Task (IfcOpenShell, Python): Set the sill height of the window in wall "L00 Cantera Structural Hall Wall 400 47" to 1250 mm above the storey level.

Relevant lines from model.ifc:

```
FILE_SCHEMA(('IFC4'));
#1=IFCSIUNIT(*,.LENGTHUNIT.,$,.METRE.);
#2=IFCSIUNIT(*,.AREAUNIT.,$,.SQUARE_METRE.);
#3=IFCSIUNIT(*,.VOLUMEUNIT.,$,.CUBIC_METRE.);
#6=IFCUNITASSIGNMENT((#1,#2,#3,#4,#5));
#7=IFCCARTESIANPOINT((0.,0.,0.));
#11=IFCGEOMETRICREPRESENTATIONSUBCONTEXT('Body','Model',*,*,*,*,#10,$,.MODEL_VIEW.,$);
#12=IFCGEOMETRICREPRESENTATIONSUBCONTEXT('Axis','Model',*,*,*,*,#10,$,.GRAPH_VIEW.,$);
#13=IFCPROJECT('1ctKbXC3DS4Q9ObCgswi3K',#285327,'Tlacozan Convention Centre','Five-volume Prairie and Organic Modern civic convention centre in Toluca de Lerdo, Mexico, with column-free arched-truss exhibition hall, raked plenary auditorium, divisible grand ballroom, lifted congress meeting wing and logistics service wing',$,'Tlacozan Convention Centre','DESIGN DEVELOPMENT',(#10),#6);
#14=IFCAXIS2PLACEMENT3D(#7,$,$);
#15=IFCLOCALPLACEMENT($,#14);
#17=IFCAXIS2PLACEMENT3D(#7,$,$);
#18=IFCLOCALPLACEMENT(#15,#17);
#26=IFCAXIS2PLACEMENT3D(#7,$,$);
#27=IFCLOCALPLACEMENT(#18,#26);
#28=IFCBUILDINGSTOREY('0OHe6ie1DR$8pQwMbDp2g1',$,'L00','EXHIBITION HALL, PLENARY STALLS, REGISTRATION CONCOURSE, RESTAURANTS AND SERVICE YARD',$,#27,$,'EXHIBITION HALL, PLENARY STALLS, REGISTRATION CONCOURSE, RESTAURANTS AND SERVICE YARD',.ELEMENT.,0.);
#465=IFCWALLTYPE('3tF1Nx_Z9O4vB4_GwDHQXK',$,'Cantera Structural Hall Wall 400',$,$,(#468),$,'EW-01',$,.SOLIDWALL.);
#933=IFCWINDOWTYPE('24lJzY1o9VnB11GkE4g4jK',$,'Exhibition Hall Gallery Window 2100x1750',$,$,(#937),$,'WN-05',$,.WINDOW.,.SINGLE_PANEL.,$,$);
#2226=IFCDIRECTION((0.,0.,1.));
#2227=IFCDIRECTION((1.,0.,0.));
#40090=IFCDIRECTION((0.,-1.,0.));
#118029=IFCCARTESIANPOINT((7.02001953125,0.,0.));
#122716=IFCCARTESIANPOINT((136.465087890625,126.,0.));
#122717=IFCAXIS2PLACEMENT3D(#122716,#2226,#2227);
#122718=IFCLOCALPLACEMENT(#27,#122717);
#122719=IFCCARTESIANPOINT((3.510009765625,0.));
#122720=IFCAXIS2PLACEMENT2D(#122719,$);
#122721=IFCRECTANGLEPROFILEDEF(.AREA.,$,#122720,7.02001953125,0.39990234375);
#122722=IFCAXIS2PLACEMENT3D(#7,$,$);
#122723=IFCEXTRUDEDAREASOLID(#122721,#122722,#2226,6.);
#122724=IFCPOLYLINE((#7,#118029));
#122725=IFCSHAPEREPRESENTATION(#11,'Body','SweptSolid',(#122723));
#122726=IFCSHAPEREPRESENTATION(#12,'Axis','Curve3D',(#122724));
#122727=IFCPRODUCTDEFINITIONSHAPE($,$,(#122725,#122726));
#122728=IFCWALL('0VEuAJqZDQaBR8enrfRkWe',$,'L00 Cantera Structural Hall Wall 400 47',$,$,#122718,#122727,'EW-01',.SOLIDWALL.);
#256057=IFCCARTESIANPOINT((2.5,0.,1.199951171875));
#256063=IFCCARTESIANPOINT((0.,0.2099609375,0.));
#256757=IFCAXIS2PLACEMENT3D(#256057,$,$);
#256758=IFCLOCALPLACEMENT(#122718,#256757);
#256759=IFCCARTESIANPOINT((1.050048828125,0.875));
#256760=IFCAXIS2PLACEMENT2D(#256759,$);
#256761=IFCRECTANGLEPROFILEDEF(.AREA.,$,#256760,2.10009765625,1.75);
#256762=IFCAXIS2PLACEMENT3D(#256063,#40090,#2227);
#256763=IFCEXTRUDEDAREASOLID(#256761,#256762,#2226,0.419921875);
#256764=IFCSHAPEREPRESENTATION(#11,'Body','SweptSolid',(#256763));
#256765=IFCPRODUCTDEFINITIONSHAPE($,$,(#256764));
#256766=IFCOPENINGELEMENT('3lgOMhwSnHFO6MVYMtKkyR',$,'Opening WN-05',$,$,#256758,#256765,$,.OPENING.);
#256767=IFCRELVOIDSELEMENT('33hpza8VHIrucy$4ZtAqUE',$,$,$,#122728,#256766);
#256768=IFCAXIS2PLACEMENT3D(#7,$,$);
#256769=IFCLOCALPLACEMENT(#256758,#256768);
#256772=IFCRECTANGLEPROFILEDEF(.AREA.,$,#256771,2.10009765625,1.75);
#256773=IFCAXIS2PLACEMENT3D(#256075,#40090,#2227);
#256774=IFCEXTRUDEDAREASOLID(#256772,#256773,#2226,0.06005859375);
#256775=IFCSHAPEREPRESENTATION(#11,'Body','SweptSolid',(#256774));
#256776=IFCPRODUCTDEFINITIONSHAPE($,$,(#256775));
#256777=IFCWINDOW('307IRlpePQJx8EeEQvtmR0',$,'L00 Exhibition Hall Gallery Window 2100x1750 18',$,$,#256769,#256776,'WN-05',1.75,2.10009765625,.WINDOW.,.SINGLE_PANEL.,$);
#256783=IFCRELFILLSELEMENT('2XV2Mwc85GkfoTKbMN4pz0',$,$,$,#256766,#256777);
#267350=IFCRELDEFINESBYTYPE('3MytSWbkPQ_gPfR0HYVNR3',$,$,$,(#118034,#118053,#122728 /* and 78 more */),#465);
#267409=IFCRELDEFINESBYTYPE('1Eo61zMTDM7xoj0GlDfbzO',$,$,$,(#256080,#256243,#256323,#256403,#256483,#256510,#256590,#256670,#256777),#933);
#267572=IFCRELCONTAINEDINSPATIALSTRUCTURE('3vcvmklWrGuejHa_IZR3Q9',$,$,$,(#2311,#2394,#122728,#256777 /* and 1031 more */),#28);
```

```python
import numpy as np
import ifcopenshell
import ifcopenshell.api.geometry
import ifcopenshell.geom
import ifcopenshell.util.element
import ifcopenshell.util.placement
import ifcopenshell.util.shape
import ifcopenshell.util.unit

model = ifcopenshell.open("model.ifc")
unit_scale = ifcopenshell.util.unit.calculate_unit_scale(model)

window = model.by_guid("307IRlpePQJx8EeEQvtmR0")
opening = window.FillsVoids[0].RelatingOpeningElement
storey = ifcopenshell.util.element.get_container(window, ifc_class="IfcBuildingStorey")
level = ifcopenshell.util.placement.get_local_placement(storey.ObjectPlacement)[2, 3]

# The opening's origin need not be at the sill, so measure its lowest point.
shape = ifcopenshell.geom.create_shape(ifcopenshell.geom.settings(), opening)
bottom = ifcopenshell.util.shape.get_shape_bottom_elevation(shape, shape.geometry) / unit_scale
dz = level + 1.25 / unit_scale - bottom

shift = np.array([0.0, 0.0, dz])
# The window is placed relative to its opening, so it follows when the opening moves.
matrix = ifcopenshell.util.placement.get_local_placement(opening.ObjectPlacement)
matrix[:3, 3] += shift
ifcopenshell.api.geometry.edit_object_placement(
    model, product=opening, matrix=matrix, is_si=False, should_transform_children=True
)

print(f"moved by {dz * unit_scale:+.3f} m")

model.write("model_updated.ifc")
```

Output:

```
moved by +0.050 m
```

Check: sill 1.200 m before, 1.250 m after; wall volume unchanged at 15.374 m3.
